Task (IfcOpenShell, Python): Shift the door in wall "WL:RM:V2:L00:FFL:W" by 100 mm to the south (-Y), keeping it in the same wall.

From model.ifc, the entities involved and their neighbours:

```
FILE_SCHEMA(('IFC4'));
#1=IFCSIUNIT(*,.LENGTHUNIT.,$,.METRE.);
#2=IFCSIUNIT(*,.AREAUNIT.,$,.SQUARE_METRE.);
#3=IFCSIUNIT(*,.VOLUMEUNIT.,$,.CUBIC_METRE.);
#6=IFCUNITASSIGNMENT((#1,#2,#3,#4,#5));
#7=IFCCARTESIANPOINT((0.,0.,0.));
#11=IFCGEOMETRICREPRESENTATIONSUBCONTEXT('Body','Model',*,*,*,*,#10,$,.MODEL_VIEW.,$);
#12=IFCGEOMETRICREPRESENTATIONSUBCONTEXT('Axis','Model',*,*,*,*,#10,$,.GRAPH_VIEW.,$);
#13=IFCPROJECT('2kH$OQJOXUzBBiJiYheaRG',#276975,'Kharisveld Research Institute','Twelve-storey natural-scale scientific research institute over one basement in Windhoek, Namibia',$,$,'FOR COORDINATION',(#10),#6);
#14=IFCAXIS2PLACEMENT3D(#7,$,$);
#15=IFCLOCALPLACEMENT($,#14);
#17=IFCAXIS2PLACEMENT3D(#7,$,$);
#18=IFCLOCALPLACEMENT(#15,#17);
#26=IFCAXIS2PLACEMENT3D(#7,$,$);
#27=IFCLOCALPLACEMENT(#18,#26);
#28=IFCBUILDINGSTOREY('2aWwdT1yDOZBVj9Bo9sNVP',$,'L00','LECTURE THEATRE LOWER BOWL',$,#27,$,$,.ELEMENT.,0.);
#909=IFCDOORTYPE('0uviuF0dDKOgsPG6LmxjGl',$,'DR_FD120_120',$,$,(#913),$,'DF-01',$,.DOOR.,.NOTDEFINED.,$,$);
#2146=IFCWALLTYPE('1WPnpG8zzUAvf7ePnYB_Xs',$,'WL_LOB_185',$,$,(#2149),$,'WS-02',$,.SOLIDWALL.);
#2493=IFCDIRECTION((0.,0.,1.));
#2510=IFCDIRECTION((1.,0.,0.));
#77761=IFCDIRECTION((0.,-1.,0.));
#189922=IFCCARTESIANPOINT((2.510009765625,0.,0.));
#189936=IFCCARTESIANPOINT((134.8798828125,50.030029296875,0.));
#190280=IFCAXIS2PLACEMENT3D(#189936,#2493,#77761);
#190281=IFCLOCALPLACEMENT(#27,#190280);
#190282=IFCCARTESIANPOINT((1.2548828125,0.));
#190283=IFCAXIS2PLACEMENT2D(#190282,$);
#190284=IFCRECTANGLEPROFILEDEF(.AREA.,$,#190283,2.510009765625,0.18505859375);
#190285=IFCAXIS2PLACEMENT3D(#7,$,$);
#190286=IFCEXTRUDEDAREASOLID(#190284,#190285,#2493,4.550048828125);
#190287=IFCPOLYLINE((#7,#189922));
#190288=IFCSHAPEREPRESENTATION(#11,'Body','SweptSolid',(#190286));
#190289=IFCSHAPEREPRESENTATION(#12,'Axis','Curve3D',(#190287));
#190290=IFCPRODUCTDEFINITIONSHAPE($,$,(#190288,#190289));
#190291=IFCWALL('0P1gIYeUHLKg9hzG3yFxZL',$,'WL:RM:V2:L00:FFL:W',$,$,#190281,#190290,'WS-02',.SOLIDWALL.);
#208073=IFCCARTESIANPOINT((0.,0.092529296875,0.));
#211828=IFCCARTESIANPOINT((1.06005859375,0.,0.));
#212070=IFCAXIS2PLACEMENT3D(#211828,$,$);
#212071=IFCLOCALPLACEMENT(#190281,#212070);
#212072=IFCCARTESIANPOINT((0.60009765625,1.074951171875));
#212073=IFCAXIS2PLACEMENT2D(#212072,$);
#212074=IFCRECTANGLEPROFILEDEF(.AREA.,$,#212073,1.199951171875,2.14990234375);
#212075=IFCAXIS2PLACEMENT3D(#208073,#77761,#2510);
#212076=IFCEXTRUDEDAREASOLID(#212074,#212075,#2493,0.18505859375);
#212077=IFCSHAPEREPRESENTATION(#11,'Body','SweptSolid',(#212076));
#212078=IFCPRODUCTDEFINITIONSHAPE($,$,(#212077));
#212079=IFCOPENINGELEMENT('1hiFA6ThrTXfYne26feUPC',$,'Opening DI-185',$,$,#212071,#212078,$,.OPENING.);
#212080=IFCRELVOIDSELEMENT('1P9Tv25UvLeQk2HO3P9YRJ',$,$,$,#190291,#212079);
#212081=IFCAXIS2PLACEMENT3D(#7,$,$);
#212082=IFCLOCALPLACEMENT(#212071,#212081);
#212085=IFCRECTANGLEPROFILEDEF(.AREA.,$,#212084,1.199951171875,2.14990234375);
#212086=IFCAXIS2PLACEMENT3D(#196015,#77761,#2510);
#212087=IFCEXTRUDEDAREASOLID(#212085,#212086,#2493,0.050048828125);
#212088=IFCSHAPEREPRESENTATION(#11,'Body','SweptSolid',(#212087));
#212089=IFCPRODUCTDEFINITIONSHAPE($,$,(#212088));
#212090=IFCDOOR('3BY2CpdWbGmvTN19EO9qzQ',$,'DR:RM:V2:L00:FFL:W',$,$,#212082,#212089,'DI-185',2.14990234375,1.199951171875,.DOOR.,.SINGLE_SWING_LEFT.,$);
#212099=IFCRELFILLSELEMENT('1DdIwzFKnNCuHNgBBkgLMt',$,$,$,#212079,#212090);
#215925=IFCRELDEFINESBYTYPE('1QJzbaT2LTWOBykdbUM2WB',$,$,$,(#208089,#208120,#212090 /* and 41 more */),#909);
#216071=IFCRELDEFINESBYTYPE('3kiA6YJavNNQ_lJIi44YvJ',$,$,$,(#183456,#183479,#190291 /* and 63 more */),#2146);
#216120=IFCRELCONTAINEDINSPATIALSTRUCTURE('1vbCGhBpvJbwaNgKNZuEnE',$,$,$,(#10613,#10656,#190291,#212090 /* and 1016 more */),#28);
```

```python
import ifcopenshell
import ifcopenshell.api.geometry
import ifcopenshell.util.placement

model = ifcopenshell.open("model.ifc")

door = model.by_id(212090)
opening = door.FillsVoids[0].RelatingOpeningElement
wall = opening.VoidsElements[0].RelatingBuildingElement

wall_matrix = ifcopenshell.util.placement.get_local_placement(wall.ObjectPlacement)
shift = wall_matrix[:3, 0] * 0.1
before = ifcopenshell.util.placement.get_local_placement(door.ObjectPlacement)[:3, 3].copy()

# The door is placed relative to its opening, so it follows when the opening moves.
matrix = ifcopenshell.util.placement.get_local_placement(opening.ObjectPlacement)
matrix[:3, 3] += shift
ifcopenshell.api.geometry.edit_object_placement(
    model, product=opening, matrix=matrix, is_si=False, should_transform_children=True
)

after = ifcopenshell.util.placement.get_local_placement(door.ObjectPlacement)[:3, 3]
print("door moved by", (after - before).round(3) + 0.0)

model.write("model_rev.ifc")
```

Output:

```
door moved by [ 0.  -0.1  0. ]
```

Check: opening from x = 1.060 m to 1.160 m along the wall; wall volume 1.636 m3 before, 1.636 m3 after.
